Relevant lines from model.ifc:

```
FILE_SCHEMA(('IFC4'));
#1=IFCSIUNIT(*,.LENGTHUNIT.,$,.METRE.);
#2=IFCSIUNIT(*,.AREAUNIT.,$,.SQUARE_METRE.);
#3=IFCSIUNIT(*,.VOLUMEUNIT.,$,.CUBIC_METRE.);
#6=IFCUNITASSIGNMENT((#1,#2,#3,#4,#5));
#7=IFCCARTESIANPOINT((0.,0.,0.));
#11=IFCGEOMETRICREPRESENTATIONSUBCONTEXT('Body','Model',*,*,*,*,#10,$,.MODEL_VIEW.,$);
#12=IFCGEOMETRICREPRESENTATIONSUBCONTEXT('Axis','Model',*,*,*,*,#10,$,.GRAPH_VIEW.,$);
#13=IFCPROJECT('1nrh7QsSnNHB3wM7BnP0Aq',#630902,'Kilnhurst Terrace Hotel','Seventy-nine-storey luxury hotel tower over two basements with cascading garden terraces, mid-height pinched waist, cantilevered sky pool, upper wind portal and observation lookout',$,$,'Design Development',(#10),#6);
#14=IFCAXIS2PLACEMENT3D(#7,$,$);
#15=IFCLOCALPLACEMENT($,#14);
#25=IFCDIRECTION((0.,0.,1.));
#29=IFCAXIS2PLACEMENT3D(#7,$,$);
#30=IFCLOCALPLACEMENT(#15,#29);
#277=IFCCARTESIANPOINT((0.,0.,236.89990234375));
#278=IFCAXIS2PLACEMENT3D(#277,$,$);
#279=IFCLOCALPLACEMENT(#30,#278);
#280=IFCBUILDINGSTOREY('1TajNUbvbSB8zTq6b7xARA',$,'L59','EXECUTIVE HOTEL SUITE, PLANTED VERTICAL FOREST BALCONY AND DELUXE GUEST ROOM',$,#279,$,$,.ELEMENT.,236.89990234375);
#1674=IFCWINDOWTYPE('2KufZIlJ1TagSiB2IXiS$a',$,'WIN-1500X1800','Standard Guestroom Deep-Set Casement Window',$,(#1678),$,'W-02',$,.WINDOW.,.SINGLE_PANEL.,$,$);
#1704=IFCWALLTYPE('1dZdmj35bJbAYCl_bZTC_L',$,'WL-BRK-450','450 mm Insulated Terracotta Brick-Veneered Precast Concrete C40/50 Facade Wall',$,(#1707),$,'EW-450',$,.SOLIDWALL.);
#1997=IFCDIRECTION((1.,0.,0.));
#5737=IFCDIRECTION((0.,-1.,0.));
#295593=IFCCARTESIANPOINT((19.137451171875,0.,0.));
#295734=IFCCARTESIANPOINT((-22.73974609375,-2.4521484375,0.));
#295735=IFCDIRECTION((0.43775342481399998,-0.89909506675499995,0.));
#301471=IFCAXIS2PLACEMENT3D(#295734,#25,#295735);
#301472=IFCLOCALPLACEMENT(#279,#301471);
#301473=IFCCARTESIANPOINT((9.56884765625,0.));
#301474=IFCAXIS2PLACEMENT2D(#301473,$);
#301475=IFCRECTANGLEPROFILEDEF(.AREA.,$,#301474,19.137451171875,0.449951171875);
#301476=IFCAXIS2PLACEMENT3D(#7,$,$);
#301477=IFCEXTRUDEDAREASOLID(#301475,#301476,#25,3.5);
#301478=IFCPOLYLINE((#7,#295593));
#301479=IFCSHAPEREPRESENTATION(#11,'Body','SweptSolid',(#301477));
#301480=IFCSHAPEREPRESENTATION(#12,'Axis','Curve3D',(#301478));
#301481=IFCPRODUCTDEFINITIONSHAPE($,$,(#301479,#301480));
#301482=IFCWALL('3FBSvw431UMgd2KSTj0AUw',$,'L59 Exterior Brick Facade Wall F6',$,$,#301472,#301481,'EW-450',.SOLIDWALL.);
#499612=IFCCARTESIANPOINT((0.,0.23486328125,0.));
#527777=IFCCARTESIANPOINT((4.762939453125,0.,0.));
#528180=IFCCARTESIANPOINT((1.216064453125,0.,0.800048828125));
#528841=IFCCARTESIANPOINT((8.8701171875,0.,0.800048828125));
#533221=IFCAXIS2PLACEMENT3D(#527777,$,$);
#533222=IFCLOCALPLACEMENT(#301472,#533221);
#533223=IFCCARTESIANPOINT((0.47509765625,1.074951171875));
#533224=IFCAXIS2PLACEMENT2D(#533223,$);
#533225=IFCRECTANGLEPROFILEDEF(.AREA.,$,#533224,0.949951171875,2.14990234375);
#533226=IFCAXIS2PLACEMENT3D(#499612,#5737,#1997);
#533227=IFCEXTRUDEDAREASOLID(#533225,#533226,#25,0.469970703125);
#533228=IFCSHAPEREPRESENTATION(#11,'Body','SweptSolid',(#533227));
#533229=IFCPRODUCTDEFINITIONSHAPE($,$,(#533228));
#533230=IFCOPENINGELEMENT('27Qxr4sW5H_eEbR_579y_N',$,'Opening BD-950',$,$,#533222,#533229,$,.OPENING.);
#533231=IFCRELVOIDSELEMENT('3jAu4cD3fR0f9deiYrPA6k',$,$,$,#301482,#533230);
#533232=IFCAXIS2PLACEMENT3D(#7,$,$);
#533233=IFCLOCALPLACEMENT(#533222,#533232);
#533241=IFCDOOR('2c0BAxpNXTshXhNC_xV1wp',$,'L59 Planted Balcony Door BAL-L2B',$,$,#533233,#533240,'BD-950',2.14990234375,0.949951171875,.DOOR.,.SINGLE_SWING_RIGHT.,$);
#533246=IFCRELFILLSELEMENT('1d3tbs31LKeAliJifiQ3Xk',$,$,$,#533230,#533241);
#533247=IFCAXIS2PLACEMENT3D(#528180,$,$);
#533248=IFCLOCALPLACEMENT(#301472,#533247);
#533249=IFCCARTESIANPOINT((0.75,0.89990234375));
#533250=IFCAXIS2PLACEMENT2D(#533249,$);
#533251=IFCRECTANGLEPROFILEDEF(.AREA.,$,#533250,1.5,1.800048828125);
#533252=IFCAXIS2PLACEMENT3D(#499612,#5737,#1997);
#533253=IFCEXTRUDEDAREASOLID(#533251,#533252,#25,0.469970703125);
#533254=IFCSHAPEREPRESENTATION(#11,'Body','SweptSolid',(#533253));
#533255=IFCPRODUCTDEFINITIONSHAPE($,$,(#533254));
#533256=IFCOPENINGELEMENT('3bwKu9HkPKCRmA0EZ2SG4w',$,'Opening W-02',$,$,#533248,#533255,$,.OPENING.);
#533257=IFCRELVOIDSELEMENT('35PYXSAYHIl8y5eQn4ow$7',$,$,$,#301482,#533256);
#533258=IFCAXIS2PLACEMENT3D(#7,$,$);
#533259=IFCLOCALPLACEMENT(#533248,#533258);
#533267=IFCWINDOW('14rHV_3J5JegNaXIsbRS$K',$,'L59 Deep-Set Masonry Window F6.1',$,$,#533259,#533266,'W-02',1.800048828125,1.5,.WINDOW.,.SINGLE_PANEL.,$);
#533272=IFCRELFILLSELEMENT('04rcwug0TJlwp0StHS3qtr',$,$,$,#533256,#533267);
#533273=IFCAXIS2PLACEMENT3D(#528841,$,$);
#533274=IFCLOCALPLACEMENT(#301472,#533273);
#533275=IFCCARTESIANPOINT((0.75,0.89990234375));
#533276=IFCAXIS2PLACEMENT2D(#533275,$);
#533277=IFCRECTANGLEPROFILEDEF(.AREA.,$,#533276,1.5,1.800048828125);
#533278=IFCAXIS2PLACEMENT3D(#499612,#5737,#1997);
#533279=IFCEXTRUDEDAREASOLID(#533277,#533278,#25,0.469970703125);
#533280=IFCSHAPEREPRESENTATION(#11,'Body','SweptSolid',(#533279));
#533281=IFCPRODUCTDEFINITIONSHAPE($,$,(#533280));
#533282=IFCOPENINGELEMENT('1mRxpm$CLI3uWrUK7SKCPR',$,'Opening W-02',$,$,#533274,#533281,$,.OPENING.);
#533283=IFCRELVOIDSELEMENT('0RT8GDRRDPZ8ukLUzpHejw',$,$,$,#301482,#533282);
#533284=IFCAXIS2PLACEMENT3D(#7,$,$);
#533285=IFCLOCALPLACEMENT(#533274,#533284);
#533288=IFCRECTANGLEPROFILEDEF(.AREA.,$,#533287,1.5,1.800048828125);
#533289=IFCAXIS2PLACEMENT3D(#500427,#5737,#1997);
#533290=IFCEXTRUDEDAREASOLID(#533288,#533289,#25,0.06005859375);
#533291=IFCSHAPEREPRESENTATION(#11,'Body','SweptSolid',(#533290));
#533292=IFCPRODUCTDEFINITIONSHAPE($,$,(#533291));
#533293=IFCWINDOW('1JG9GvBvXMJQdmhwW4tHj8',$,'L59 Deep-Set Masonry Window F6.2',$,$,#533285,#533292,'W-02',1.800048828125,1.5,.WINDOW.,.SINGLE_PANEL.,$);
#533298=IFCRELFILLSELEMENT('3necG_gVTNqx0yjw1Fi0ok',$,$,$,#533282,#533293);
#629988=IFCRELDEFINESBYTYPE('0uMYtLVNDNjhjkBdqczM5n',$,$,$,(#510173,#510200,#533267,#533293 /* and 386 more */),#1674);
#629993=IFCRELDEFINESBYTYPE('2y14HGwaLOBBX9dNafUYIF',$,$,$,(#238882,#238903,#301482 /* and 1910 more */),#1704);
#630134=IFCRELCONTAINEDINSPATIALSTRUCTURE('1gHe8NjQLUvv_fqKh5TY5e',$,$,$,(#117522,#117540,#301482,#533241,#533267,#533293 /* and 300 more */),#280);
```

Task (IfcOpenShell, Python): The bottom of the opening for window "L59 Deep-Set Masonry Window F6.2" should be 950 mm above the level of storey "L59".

```python
import numpy as np
import ifcopenshell
import ifcopenshell.api.geometry
import ifcopenshell.geom
import ifcopenshell.util.element
import ifcopenshell.util.placement
import ifcopenshell.util.shape
import ifcopenshell.util.unit

model = ifcopenshell.open("model.ifc")
unit_scale = ifcopenshell.util.unit.calculate_unit_scale(model)

window = model.by_id(533293)
opening = window.FillsVoids[0].RelatingOpeningElement
storey = ifcopenshell.util.element.get_container(window, ifc_class="IfcBuildingStorey")
level = ifcopenshell.util.placement.get_local_placement(storey.ObjectPlacement)[2, 3]

# The opening's origin need not be at the sill, so measure its lowest point.
shape = ifcopenshell.geom.create_shape(ifcopenshell.geom.settings(), opening)
bottom = ifcopenshell.util.shape.get_shape_bottom_elevation(shape, shape.geometry) / unit_scale
dz = level + 0.95 / unit_scale - bottom

shift = np.array([0.0, 0.0, dz])
# The window is placed relative to its opening, so it follows when the opening moves.
matrix = ifcopenshell.util.placement.get_local_placement(opening.ObjectPlacement)
matrix[:3, 3] += shift
ifcopenshell.api.geometry.edit_object_placement(
    model, product=opening, matrix=matrix, is_si=False, should_transform_children=True
)

print(f"moved by {dz * unit_scale:+.3f} m")

model.write("model_v2.ifc")
```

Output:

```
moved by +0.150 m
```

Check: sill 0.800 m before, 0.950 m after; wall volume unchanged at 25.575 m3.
